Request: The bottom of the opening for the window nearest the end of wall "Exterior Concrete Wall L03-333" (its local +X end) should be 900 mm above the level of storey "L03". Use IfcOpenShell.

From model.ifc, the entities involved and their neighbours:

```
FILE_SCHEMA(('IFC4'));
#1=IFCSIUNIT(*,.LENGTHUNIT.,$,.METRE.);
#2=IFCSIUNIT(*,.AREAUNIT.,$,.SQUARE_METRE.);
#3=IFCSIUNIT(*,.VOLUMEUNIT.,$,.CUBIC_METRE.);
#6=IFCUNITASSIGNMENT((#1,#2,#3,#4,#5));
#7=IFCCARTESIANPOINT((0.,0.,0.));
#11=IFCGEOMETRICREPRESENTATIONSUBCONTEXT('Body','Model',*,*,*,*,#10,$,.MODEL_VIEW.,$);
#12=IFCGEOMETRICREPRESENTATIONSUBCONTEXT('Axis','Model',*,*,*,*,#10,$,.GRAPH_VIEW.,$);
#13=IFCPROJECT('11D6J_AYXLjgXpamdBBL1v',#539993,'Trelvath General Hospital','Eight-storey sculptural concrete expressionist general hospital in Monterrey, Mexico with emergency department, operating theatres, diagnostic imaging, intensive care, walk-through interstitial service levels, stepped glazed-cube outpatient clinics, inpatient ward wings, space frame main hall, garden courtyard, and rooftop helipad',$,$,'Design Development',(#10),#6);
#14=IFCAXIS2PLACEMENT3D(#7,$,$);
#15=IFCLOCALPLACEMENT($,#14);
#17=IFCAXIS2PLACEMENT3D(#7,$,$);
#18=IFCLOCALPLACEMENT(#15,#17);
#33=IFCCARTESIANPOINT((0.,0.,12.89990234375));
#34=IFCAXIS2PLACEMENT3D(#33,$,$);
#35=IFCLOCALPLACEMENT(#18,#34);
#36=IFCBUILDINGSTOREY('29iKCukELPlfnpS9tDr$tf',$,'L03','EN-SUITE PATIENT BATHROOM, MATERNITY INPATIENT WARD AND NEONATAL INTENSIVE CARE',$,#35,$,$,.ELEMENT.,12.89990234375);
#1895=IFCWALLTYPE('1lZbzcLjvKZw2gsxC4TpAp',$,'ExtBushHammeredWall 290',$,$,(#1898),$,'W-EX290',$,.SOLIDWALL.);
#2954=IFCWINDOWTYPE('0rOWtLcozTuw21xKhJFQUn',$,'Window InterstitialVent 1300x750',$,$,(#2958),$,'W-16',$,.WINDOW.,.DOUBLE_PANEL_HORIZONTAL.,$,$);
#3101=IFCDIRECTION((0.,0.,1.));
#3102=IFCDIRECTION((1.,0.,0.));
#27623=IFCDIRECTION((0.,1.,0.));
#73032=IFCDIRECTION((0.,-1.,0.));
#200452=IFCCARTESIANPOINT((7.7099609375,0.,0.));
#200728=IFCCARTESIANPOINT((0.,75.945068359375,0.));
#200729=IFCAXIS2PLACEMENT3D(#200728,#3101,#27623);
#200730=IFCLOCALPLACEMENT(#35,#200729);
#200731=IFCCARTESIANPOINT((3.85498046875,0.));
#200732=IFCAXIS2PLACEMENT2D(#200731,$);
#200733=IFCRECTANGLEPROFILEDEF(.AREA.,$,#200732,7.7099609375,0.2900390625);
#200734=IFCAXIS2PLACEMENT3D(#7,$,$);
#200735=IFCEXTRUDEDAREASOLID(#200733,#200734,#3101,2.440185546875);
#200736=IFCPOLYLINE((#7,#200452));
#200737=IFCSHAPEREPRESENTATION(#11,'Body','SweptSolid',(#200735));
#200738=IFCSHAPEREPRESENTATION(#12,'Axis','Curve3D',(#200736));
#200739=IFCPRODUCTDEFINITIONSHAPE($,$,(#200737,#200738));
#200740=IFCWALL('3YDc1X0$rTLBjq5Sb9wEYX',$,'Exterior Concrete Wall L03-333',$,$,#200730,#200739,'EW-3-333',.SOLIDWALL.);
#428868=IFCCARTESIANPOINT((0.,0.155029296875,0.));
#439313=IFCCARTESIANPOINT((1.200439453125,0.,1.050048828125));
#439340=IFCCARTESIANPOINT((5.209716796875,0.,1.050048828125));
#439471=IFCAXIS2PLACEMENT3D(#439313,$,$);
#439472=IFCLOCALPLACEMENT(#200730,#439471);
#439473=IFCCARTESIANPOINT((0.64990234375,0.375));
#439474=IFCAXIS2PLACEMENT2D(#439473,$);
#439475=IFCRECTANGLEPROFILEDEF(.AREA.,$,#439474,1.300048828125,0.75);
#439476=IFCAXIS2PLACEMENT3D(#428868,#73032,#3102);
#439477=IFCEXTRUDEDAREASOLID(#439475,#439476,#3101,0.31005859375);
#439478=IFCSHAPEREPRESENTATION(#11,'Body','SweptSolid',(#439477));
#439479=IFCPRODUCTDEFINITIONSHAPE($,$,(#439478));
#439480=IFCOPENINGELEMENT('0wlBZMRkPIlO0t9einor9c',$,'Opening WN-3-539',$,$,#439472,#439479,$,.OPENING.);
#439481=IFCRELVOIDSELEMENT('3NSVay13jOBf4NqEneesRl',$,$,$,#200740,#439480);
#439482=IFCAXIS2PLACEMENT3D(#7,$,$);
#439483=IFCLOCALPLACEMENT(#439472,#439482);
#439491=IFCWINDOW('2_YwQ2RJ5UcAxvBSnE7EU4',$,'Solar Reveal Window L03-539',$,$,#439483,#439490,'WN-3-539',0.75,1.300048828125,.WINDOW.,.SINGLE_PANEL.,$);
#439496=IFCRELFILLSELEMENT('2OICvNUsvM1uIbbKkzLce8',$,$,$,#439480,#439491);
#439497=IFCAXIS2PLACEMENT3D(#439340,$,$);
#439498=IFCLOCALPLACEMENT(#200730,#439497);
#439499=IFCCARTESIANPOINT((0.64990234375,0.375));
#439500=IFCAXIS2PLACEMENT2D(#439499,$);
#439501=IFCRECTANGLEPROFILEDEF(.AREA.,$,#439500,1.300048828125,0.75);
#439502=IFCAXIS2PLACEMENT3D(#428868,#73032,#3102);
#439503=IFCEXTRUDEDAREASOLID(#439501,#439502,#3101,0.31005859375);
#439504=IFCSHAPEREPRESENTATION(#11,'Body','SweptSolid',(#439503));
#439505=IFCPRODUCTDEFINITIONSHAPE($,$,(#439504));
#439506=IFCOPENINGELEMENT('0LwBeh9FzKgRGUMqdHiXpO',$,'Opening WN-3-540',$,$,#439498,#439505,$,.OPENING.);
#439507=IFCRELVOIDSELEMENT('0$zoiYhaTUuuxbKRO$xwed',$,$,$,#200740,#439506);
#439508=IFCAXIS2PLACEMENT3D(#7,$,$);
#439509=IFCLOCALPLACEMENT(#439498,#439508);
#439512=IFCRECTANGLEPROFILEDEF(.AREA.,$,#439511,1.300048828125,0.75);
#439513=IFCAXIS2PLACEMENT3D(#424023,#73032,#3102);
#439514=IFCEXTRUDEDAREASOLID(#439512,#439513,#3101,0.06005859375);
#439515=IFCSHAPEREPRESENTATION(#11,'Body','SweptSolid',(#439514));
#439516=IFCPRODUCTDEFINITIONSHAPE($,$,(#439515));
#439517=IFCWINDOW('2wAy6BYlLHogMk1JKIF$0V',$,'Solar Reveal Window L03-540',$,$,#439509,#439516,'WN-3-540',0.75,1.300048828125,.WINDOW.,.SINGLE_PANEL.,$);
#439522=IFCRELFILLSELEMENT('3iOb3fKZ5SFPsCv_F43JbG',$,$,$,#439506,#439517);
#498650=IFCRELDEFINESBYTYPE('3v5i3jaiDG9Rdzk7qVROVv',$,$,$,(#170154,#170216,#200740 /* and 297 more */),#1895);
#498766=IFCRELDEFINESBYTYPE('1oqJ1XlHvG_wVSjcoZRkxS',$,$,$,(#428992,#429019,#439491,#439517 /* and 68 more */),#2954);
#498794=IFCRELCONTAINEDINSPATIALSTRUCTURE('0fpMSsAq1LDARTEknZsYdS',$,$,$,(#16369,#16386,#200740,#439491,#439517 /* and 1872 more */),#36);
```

```python
import numpy as np
import ifcopenshell
import ifcopenshell.api.geometry
import ifcopenshell.geom
import ifcopenshell.util.element
import ifcopenshell.util.placement
import ifcopenshell.util.shape
import ifcopenshell.util.unit

model = ifcopenshell.open("model.ifc")
unit_scale = ifcopenshell.util.unit.calculate_unit_scale(model)

window = model.by_guid("2wAy6BYlLHogMk1JKIF$0V")
opening = window.FillsVoids[0].RelatingOpeningElement
storey = ifcopenshell.util.element.get_container(window, ifc_class="IfcBuildingStorey")
level = ifcopenshell.util.placement.get_local_placement(storey.ObjectPlacement)[2, 3]

# The opening's origin need not be at the sill, so measure its lowest point.
shape = ifcopenshell.geom.create_shape(ifcopenshell.geom.settings(), opening)
bottom = ifcopenshell.util.shape.get_shape_bottom_elevation(shape, shape.geometry) / unit_scale
dz = level + 0.9 - bottom

shift = np.array([0.0, 0.0, dz])
# The window is placed relative to its opening, so it follows when the opening moves.
matrix = ifcopenshell.util.placement.get_local_placement(opening.ObjectPlacement)
matrix[:3, 3] += shift
ifcopenshell.api.geometry.edit_object_placement(
    model, product=opening, matrix=matrix, is_si=False, should_transform_children=True
)

print(f"moved by {dz * unit_scale:+.3f} m")

model.write("model_v2.ifc")
```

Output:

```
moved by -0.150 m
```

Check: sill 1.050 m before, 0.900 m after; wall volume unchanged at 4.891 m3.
